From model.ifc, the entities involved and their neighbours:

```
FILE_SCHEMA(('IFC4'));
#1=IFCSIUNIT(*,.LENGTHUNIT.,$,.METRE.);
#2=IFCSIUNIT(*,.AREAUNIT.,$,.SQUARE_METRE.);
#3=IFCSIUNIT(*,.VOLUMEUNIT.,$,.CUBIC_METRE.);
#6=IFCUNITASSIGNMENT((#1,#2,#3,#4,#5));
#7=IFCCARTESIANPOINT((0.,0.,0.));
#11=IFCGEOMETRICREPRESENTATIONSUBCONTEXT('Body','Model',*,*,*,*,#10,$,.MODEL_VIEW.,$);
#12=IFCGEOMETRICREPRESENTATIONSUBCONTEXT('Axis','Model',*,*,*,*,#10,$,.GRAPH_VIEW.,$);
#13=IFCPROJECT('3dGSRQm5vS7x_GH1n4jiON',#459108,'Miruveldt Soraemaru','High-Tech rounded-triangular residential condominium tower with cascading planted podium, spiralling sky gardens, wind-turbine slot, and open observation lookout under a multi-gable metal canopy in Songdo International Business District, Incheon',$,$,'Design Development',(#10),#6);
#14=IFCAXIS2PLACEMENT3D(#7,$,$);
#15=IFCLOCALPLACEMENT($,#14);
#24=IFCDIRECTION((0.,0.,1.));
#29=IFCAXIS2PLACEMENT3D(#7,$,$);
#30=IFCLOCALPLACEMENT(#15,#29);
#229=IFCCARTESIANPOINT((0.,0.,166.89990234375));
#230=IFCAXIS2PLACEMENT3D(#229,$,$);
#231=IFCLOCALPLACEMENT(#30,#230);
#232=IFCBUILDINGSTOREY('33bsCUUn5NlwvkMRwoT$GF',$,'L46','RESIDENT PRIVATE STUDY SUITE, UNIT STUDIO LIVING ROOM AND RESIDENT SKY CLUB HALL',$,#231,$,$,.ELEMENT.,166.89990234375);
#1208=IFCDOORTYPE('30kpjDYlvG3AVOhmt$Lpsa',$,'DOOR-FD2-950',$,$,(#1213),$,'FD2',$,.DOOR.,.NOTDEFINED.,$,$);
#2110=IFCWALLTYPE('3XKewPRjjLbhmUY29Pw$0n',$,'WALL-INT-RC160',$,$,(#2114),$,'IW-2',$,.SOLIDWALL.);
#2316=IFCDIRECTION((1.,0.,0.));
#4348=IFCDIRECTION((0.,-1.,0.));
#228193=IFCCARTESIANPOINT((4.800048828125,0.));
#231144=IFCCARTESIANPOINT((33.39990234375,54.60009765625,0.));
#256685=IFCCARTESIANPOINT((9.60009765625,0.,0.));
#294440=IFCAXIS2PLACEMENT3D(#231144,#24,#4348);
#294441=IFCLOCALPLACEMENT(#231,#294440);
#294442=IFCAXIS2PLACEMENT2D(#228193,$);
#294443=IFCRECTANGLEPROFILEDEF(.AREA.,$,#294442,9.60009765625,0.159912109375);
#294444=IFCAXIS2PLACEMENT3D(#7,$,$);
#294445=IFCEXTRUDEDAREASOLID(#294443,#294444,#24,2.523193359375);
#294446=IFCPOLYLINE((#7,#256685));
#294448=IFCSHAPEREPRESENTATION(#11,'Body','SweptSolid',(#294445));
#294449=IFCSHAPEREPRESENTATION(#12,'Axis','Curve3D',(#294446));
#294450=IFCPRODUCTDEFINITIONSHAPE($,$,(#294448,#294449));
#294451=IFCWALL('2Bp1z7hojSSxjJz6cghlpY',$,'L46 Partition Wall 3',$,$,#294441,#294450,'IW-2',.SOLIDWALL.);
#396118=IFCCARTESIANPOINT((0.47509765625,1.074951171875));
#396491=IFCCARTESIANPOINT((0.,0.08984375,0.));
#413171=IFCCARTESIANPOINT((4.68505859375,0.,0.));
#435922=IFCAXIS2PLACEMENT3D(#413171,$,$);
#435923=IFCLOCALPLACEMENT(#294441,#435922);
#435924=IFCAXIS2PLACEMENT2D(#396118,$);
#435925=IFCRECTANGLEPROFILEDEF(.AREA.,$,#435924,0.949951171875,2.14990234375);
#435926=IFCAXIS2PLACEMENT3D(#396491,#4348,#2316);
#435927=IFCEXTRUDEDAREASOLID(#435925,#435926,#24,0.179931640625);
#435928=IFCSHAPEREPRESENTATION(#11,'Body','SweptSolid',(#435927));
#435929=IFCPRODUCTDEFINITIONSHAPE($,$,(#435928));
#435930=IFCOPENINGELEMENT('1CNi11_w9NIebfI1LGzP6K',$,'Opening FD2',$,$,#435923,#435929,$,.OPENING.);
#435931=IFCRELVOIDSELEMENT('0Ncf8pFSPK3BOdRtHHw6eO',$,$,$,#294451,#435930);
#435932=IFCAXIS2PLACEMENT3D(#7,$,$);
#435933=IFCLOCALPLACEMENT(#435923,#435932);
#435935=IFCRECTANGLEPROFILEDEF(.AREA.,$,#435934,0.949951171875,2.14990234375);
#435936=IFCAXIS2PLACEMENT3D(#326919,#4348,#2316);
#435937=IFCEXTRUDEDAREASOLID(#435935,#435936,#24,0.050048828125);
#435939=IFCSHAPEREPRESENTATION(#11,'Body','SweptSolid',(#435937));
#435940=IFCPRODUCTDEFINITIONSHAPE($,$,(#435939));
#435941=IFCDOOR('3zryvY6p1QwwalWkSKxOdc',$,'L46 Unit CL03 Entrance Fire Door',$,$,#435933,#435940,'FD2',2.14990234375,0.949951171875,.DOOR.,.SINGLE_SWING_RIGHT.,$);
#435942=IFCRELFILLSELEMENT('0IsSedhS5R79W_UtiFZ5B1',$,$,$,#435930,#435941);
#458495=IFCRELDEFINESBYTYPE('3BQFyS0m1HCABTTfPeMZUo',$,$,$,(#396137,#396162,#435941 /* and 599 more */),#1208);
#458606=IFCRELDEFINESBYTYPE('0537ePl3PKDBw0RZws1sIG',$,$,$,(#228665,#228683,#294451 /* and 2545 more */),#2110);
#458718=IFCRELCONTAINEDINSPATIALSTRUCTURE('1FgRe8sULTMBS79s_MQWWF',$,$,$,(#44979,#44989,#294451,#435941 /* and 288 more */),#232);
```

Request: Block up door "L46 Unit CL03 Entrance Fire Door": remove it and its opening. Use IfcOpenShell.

```python
import ifcopenshell
import ifcopenshell.api.feature
import ifcopenshell.api.root
import ifcopenshell.geom
import ifcopenshell.util.shape

model = ifcopenshell.open("model.ifc")
settings = ifcopenshell.geom.settings()


def volume(element):
    """Net volume in cubic metres, openings subtracted."""
    shape = ifcopenshell.geom.create_shape(settings, element)
    return ifcopenshell.util.shape.get_volume(shape.geometry)


door = model.by_guid("3zryvY6p1QwwalWkSKxOdc")
opening = door.FillsVoids[0].RelatingOpeningElement
wall = opening.VoidsElements[0].RelatingBuildingElement
before = volume(wall)

ifcopenshell.api.root.remove_product(model, product=door)
ifcopenshell.api.feature.remove_feature(model, feature=opening)

after = volume(wall)

print(f"wall volume {before:.3f} -> {after:.3f} m3")

model.write("model-out.ifc")
```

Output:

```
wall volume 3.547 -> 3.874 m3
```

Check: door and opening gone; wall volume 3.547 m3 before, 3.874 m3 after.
